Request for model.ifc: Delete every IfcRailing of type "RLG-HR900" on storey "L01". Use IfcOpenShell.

First a look at what the model holds.

```python
import ifcopenshell
import ifcopenshell.util.element

model = ifcopenshell.open("model.ifc")
print(model.schema)
storey = next(s for s in model.by_type("IfcBuildingStorey") if s.Name == "L01")
railings = [e for e in ifcopenshell.util.element.get_decomposition(storey) if e.is_a("IfcRailing")]
seen = {}
for e in railings:
    element_type = ifcopenshell.util.element.get_type(e)
    name = element_type.Name if element_type not in (None, e) else None
    seen[name] = seen.get(name, 0) + 1
for name, count in sorted(seen.items(), key=str):
    print(count, "x", name)
```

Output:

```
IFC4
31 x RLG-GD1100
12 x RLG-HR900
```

```python
import ifcopenshell
import ifcopenshell.api.root
import ifcopenshell.util.element

model = ifcopenshell.open("model.ifc")

storey = next(s for s in model.by_type("IfcBuildingStorey") if s.Name == "L01")
railings = [e for e in ifcopenshell.util.element.get_decomposition(storey) if e.is_a("IfcRailing")]
targets = [e for e in railings if (t := ifcopenshell.util.element.get_type(e)) not in (None, e) and t.Name == "RLG-HR900"]

for e in targets:
    ifcopenshell.api.root.remove_product(model, product=e)
print(len(targets), "removed")

model.write("model_v2.ifc")
```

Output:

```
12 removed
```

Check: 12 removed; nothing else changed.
